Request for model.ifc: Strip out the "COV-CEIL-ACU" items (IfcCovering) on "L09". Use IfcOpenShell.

First a look at what the model holds.

```python
import ifcopenshell
import ifcopenshell.util.element

model = ifcopenshell.open("model.ifc")
print(model.schema)
storey = next(s for s in model.by_type("IfcBuildingStorey") if s.Name == "L09")
coverings = [e for e in ifcopenshell.util.element.get_decomposition(storey) if e.is_a("IfcCovering")]
seen = {}
for e in coverings:
    element_type = ifcopenshell.util.element.get_type(e)
    name = element_type.Name if element_type not in (None, e) else None
    seen[name] = seen.get(name, 0) + 1
for name, count in sorted(seen.items(), key=str):
    print(count, "x", name)
```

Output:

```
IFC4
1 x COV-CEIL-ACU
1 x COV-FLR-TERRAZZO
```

```python
import ifcopenshell
import ifcopenshell.api.root
import ifcopenshell.util.element

model = ifcopenshell.open("model.ifc")

storey = next(s for s in model.by_type("IfcBuildingStorey") if s.Name == "L09")
coverings = [e for e in ifcopenshell.util.element.get_decomposition(storey) if e.is_a("IfcCovering")]
targets = [e for e in coverings if (t := ifcopenshell.util.element.get_type(e)) not in (None, e) and t.Name == "COV-CEIL-ACU"]

for e in targets:
    ifcopenshell.api.root.remove_product(model, product=e)
print(len(targets), "removed")

model.write("model_updated.ifc")
```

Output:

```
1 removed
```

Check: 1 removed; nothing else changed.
